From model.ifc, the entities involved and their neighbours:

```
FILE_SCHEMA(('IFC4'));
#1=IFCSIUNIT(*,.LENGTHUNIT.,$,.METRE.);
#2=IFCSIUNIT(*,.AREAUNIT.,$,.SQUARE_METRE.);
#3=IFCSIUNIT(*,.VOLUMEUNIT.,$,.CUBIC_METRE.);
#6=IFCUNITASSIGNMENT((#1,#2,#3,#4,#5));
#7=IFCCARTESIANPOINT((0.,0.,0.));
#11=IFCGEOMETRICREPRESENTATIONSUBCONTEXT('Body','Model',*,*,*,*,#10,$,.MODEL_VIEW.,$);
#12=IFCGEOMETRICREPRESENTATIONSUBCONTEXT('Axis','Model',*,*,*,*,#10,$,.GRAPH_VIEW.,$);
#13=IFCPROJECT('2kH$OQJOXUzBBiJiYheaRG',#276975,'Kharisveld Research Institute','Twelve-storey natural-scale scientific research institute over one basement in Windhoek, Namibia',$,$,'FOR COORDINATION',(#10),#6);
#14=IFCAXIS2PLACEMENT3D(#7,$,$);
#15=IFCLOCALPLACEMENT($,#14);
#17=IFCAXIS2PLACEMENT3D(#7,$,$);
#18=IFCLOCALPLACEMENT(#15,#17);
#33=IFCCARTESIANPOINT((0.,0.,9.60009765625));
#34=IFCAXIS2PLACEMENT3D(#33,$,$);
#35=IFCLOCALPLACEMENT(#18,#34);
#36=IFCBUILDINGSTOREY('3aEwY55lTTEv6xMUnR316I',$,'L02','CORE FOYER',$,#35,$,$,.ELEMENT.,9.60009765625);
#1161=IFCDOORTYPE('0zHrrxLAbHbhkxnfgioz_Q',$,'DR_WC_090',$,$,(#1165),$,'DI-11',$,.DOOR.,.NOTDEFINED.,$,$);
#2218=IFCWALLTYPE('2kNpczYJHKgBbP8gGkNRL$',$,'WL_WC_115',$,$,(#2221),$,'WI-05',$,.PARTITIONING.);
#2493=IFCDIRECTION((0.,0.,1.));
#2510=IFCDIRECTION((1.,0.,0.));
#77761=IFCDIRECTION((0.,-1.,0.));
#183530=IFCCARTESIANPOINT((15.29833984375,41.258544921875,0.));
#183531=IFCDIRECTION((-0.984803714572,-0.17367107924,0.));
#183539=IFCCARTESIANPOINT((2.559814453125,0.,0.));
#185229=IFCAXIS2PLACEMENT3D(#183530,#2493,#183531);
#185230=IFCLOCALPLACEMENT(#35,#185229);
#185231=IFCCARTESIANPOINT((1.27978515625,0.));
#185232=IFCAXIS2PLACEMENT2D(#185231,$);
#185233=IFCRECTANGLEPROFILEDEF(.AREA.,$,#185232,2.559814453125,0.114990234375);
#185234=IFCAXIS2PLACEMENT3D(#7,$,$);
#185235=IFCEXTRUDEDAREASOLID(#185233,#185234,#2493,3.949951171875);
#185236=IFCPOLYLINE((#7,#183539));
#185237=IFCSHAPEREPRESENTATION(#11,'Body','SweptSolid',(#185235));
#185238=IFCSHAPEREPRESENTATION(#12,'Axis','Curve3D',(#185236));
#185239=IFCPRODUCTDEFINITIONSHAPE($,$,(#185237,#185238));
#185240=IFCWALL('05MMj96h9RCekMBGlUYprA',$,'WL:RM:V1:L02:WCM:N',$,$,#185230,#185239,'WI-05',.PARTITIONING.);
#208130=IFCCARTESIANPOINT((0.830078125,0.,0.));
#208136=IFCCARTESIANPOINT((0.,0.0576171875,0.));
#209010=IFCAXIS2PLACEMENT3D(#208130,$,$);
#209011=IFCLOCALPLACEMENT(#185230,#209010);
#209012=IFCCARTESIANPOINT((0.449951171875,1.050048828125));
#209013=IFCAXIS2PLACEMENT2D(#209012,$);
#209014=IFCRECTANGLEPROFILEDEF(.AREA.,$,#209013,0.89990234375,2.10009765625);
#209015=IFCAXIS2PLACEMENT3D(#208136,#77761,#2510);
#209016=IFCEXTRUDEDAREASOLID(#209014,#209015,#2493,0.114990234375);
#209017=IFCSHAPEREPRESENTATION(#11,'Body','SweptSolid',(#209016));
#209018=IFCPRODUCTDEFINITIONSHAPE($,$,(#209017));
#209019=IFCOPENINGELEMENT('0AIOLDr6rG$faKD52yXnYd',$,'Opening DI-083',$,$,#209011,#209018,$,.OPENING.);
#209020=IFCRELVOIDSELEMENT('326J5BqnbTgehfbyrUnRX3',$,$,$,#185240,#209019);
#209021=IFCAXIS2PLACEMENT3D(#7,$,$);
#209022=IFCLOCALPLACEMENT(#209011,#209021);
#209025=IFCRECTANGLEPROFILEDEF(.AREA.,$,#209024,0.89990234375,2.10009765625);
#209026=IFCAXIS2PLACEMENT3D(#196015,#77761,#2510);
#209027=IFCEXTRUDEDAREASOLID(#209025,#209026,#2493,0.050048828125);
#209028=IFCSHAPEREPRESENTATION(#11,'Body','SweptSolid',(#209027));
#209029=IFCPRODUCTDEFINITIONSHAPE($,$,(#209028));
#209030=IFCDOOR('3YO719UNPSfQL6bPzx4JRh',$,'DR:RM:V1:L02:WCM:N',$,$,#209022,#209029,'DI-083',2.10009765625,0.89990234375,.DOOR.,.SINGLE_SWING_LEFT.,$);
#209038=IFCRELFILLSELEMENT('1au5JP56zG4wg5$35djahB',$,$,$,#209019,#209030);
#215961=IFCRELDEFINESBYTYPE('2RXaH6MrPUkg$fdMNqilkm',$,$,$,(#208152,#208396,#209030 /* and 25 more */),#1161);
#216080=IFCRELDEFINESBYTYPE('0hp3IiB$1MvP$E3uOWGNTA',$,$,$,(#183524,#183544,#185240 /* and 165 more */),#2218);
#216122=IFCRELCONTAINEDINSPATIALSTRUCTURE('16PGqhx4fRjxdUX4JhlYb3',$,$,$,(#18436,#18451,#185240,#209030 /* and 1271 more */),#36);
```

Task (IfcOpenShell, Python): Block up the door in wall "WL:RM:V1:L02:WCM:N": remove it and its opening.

```python
import ifcopenshell
import ifcopenshell.api.feature
import ifcopenshell.api.root
import ifcopenshell.geom
import ifcopenshell.util.shape

model = ifcopenshell.open("model.ifc")
settings = ifcopenshell.geom.settings()


def volume(element):
    """Net volume in cubic metres, openings subtracted."""
    shape = ifcopenshell.geom.create_shape(settings, element)
    return ifcopenshell.util.shape.get_volume(shape.geometry)


door = model.by_guid("3YO719UNPSfQL6bPzx4JRh")
opening = door.FillsVoids[0].RelatingOpeningElement
wall = opening.VoidsElements[0].RelatingBuildingElement
before = volume(wall)

ifcopenshell.api.root.remove_product(model, product=door)
ifcopenshell.api.feature.remove_feature(model, feature=opening)

after = volume(wall)

print(f"wall volume {before:.3f} -> {after:.3f} m3")

model.write("model_rev.ifc")
```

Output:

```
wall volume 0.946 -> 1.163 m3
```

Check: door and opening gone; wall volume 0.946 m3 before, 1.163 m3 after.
